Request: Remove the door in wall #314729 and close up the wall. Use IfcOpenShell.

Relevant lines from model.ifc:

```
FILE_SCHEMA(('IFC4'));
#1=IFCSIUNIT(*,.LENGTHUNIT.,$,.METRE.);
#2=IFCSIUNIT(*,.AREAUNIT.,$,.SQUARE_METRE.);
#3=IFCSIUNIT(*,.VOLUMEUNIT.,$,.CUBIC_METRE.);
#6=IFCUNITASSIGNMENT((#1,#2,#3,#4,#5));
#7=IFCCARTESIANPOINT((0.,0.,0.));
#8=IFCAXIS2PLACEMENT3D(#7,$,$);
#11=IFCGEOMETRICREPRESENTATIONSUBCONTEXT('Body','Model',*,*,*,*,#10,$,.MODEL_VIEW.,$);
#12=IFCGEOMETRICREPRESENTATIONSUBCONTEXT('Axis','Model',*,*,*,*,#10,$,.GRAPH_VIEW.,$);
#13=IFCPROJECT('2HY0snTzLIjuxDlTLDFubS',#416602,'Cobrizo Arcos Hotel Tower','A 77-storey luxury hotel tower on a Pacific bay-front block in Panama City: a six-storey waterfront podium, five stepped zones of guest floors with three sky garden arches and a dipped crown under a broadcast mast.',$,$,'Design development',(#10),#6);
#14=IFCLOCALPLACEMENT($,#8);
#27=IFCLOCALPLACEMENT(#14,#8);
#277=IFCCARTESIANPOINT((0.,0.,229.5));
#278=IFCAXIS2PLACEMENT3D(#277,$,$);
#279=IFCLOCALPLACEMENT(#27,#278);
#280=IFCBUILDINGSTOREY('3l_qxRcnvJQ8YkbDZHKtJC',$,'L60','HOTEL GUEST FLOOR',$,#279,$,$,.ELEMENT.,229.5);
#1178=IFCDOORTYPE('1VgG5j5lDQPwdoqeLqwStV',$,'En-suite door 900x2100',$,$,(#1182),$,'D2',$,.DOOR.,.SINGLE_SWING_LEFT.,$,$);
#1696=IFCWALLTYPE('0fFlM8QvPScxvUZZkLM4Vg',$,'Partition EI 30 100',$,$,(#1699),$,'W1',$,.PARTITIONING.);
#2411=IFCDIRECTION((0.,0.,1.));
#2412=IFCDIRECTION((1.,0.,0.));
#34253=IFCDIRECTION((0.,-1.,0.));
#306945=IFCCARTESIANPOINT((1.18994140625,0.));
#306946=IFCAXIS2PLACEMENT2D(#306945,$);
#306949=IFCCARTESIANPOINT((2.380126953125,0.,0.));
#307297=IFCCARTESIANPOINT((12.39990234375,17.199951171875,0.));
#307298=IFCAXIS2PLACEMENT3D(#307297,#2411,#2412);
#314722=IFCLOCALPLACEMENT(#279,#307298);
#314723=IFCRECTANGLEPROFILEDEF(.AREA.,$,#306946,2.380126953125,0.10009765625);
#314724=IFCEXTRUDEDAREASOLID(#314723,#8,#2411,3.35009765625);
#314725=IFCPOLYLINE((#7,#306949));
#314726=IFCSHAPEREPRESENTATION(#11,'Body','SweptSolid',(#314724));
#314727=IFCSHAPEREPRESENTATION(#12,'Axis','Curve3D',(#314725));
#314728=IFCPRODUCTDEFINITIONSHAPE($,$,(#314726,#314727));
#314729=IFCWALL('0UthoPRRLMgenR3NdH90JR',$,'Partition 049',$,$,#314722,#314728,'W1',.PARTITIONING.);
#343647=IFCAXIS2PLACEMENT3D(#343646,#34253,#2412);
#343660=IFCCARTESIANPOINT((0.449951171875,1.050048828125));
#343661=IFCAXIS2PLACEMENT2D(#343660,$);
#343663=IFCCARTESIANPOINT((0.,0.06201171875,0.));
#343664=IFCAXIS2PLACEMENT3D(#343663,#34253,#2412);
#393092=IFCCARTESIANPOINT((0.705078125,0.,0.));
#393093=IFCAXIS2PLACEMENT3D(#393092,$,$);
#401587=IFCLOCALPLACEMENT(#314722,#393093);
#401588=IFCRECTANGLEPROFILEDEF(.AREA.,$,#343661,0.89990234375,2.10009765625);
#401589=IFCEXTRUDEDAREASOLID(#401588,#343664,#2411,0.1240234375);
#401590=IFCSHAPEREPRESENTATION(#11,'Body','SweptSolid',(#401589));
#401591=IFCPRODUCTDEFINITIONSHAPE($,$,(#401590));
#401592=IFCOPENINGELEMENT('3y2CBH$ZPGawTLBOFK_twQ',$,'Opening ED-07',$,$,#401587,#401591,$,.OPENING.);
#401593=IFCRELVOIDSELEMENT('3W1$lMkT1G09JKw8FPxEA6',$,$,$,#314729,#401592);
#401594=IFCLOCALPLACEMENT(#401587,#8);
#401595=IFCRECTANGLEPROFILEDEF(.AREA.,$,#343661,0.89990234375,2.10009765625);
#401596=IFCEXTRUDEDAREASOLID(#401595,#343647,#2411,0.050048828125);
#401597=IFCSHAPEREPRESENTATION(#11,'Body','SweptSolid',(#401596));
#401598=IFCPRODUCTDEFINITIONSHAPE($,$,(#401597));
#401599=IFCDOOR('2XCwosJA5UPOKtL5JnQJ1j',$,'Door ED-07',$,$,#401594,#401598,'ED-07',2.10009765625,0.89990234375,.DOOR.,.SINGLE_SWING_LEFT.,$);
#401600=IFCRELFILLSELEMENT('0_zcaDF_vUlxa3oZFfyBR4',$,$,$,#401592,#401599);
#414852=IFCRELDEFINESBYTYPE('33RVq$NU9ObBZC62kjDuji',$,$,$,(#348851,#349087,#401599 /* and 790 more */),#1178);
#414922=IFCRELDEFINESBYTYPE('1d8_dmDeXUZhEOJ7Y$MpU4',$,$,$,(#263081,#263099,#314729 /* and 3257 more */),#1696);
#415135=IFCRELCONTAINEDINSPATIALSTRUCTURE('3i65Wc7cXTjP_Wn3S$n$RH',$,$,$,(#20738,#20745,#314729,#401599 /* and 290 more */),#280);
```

```python
import ifcopenshell
import ifcopenshell.api.feature
import ifcopenshell.api.root
import ifcopenshell.geom
import ifcopenshell.util.shape

model = ifcopenshell.open("model.ifc")
settings = ifcopenshell.geom.settings()


def volume(element):
    """Net volume in cubic metres, openings subtracted."""
    shape = ifcopenshell.geom.create_shape(settings, element)
    return ifcopenshell.util.shape.get_volume(shape.geometry)


door = model.by_guid("2XCwosJA5UPOKtL5JnQJ1j")
opening = door.FillsVoids[0].RelatingOpeningElement
wall = opening.VoidsElements[0].RelatingBuildingElement
before = volume(wall)

ifcopenshell.api.root.remove_product(model, product=door)
ifcopenshell.api.feature.remove_feature(model, feature=opening)

after = volume(wall)

print(f"wall volume {before:.3f} -> {after:.3f} m3")

model.write("model_updated.ifc")
```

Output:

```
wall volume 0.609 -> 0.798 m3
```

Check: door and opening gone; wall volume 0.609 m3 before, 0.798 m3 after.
